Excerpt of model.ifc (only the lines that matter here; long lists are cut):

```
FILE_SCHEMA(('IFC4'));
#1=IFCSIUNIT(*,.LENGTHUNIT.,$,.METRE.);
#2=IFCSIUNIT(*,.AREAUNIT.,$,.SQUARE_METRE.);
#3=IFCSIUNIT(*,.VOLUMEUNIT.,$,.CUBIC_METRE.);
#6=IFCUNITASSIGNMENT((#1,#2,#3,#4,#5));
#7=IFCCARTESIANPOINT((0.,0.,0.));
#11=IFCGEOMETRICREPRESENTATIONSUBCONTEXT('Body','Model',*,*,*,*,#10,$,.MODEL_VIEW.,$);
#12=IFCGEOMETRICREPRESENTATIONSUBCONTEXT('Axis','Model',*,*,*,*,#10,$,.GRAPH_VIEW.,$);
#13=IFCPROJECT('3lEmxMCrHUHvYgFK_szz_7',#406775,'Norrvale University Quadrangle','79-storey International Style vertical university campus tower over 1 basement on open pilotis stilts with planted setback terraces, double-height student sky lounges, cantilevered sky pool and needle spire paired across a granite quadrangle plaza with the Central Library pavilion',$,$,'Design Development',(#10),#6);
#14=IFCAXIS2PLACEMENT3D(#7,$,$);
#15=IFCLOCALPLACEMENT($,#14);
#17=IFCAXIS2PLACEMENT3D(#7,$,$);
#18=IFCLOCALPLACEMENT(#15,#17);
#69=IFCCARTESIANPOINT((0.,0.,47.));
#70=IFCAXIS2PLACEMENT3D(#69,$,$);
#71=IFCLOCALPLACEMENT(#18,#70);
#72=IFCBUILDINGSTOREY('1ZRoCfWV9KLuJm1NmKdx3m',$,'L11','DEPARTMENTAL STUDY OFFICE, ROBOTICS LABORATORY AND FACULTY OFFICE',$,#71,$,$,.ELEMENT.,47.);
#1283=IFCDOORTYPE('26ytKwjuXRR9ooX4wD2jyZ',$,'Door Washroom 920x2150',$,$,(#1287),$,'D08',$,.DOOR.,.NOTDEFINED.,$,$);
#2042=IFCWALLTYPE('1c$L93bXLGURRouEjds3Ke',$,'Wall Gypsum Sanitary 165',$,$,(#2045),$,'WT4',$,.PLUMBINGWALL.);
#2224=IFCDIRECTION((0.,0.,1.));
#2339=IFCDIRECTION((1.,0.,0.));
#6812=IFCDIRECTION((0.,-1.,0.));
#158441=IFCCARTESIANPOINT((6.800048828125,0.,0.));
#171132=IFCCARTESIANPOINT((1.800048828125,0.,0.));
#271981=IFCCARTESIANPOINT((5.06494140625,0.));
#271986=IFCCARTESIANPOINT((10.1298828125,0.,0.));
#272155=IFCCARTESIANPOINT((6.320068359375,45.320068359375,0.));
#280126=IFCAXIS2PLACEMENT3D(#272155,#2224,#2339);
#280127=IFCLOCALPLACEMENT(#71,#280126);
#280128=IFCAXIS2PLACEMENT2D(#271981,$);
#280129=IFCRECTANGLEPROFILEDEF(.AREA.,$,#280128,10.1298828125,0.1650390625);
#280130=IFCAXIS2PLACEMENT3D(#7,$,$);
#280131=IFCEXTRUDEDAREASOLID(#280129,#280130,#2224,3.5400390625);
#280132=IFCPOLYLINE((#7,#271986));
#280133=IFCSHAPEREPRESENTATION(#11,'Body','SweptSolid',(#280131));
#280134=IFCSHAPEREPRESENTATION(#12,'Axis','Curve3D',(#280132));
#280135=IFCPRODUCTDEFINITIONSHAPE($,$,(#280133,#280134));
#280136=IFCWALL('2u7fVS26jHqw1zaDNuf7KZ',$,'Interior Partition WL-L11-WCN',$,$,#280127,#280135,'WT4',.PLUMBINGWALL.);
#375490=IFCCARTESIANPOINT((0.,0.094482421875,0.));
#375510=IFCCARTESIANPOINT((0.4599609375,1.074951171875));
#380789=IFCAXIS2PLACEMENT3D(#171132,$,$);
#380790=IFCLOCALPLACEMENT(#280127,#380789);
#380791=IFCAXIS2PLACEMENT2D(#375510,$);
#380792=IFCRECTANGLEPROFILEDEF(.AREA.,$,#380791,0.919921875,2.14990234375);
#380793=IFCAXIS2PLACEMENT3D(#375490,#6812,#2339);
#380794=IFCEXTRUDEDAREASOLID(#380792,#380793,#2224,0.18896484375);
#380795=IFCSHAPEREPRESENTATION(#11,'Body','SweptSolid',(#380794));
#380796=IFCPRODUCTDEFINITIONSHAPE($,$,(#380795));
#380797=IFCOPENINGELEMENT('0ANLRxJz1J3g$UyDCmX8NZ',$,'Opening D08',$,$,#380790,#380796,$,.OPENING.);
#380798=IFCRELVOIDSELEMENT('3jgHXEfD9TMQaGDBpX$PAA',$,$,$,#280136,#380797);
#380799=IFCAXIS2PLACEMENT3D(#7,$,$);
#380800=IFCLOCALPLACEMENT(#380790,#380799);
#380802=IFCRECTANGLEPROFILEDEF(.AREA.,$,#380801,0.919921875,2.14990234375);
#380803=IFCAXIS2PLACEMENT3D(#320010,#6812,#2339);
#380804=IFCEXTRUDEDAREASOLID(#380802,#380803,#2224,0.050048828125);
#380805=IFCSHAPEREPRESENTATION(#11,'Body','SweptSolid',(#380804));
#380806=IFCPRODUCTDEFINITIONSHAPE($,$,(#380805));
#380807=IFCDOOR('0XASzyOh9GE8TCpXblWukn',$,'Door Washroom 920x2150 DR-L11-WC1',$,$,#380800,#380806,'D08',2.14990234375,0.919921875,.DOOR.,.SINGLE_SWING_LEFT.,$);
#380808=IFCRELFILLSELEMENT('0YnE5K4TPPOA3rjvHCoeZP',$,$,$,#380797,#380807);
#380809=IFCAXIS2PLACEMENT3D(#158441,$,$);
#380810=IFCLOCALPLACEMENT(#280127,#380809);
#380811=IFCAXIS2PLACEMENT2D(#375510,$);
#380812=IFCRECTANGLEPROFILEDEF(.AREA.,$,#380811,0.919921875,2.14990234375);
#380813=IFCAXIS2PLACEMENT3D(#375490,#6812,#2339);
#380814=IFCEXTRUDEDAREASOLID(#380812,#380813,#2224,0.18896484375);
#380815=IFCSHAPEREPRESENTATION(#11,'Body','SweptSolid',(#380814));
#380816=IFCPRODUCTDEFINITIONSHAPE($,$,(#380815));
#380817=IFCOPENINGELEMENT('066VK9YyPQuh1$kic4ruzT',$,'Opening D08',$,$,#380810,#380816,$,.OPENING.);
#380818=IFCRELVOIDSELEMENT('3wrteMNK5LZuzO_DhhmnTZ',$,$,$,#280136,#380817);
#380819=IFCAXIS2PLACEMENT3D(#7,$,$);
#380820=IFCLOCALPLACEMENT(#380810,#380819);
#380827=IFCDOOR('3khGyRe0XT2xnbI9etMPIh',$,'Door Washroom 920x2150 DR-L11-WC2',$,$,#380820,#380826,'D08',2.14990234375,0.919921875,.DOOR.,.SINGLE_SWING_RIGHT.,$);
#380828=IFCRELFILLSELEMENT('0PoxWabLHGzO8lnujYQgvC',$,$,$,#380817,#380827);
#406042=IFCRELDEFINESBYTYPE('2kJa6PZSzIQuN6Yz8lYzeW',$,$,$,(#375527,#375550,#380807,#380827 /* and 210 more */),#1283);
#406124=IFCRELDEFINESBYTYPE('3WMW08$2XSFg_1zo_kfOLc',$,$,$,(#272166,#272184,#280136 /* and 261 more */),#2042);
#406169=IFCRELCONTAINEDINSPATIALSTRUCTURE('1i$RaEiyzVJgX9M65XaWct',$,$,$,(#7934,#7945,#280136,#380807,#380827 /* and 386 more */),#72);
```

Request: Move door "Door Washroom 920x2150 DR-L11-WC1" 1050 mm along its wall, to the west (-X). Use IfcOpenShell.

```python
import ifcopenshell
import ifcopenshell.api.geometry
import ifcopenshell.util.placement
import ifcopenshell.util.unit

model = ifcopenshell.open("model.ifc")
unit_scale = ifcopenshell.util.unit.calculate_unit_scale(model)

door = model.by_guid("0XASzyOh9GE8TCpXblWukn")
opening = door.FillsVoids[0].RelatingOpeningElement
wall = opening.VoidsElements[0].RelatingBuildingElement

wall_matrix = ifcopenshell.util.placement.get_local_placement(wall.ObjectPlacement)
shift = wall_matrix[:3, 0] * -1.05 / unit_scale
before = ifcopenshell.util.placement.get_local_placement(door.ObjectPlacement)[:3, 3].copy()

# The door is placed relative to its opening, so it follows when the opening moves.
matrix = ifcopenshell.util.placement.get_local_placement(opening.ObjectPlacement)
matrix[:3, 3] += shift
ifcopenshell.api.geometry.edit_object_placement(
    model, product=opening, matrix=matrix, is_si=False, should_transform_children=True
)

after = ifcopenshell.util.placement.get_local_placement(door.ObjectPlacement)[:3, 3]
print("door moved by", (after - before).round(3) + 0.0)

model.write("model_edited.ifc")
```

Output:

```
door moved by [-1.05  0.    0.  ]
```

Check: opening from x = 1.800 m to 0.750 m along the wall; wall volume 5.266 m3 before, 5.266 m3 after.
